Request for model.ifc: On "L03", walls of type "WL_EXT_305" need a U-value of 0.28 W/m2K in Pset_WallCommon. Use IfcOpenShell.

First a look at what the model holds.

```python
import ifcopenshell
import ifcopenshell.util.element

model = ifcopenshell.open("model.ifc")
print(model.schema)
storey = next(s for s in model.by_type("IfcBuildingStorey") if s.Name == "L03")
walls = [e for e in ifcopenshell.util.element.get_decomposition(storey) if e.is_a("IfcWall")]
seen = {}
for e in walls:
    element_type = ifcopenshell.util.element.get_type(e)
    key = (element_type.Name if element_type != e and element_type else None, ifcopenshell.util.element.get_pset(e, "Pset_WallCommon", "ThermalTransmittance"))
    seen[key] = seen.get(key, 0) + 1
for (name, value), count in sorted(seen.items(), key=str):
    print(count, "x", name, "|", value)
```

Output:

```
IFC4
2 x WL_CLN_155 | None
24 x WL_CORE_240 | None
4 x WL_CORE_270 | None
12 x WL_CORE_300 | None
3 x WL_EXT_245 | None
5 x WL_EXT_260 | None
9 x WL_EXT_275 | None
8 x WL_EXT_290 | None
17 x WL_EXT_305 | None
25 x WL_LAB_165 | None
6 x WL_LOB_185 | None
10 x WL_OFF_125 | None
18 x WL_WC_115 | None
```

```python
import ifcopenshell
import ifcopenshell.api.pset
import ifcopenshell.util.element

model = ifcopenshell.open("model.ifc")

storey = next(s for s in model.by_type("IfcBuildingStorey") if s.Name == "L03")
walls = [e for e in ifcopenshell.util.element.get_decomposition(storey) if e.is_a("IfcWall")]

count = 0
for e in walls:
    element_type = ifcopenshell.util.element.get_type(e)
    if element_type in (None, e) or element_type.Name != "WL_EXT_305":
        continue
    # add_pset returns the element's existing set when there is one.
    pset = ifcopenshell.api.pset.add_pset(model, product=e, name="Pset_WallCommon")
    ifcopenshell.api.pset.edit_pset(model, pset=pset, properties={"ThermalTransmittance": 0.28})
    count += 1

print(count, "walls updated")

model.write("model_v2.ifc")
```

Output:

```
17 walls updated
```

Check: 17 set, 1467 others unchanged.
